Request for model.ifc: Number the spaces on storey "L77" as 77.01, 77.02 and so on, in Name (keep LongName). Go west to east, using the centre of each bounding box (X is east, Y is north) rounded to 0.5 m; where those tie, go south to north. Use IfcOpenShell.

First a look at what the model holds.

```python
import ifcopenshell
import ifcopenshell.util.element
import ifcopenshell.util.placement

model = ifcopenshell.open("model.ifc")
print(model.schema)
storey = next(s for s in model.by_type("IfcBuildingStorey") if s.Name == "L77")
spaces = [e for e in ifcopenshell.util.element.get_decomposition(storey) if e.is_a("IfcSpace")]
for e in sorted(spaces, key=lambda e: e.id()):
    origin = ifcopenshell.util.placement.get_local_placement(e.ObjectPlacement)[:3, 3]
    print(e.id(), e.Name, e.LongName, origin.round(2) + 0.0, sep=" | ")
```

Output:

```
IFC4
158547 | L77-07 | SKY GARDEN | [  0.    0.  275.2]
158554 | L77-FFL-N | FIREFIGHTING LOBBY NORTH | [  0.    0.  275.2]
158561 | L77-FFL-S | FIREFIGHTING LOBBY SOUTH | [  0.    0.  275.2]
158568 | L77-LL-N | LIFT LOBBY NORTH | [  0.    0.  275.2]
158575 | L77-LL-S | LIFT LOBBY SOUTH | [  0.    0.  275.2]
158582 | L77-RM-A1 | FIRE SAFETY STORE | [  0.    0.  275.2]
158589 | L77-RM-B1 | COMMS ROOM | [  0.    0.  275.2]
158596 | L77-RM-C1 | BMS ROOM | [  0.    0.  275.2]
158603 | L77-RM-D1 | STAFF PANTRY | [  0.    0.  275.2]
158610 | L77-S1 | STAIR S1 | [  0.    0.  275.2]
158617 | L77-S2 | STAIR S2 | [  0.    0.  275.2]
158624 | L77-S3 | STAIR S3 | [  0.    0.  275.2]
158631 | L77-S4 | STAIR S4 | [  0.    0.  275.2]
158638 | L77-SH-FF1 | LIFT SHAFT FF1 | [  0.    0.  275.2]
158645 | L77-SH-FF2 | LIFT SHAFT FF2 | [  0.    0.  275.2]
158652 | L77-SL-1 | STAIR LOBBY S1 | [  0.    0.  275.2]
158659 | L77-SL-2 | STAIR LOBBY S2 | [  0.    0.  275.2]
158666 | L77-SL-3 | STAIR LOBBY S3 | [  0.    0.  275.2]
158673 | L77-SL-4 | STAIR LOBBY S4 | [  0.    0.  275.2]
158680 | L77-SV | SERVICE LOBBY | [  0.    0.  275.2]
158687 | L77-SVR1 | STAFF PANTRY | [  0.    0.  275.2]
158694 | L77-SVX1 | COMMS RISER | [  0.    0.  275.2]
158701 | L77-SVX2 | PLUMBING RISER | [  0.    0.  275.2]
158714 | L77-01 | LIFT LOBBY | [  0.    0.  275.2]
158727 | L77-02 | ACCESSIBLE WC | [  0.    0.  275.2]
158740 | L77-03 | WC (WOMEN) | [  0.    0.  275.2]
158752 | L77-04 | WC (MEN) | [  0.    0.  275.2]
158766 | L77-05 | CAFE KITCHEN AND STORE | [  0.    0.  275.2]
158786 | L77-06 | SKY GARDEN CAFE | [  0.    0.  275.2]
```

```python
import ifcopenshell
import ifcopenshell.geom
import ifcopenshell.util.element
import ifcopenshell.util.shape

model = ifcopenshell.open("model.ifc")
settings = ifcopenshell.geom.settings()
settings.set("use-world-coords", True)


def centre(element):
    shape = ifcopenshell.geom.create_shape(settings, element)
    return ifcopenshell.util.shape.get_bbox_centroid(shape.geometry)


storey = next(s for s in model.by_type("IfcBuildingStorey") if s.Name == "L77")
spaces = [e for e in ifcopenshell.util.element.get_decomposition(storey) if e.is_a("IfcSpace")]

# Insertion points can sit at a corner or the storey origin, so sort by the geometry (in metres).
centres = {e: centre(e) for e in spaces}
spaces.sort(key=lambda e: (round(centres[e][0] / 0.5), centres[e][1]))

for i, e in enumerate(spaces, start=1):
    number = f"77.{i:02d}"
    e.Name = number
    print(e.id(), number)

model.write("model_rev.ifc")
```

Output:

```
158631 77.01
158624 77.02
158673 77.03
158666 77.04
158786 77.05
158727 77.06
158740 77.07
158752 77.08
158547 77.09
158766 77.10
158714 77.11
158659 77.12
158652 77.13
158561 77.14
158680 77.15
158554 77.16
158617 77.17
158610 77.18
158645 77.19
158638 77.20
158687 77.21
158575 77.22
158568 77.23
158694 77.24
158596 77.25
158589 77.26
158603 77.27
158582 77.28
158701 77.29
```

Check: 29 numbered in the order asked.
